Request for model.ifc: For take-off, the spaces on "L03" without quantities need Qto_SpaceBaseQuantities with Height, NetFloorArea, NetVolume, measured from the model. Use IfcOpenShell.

First a look at what the model holds.

```python
import ifcopenshell
import ifcopenshell.util.element
import ifcopenshell.util.unit

model = ifcopenshell.open("model.ifc")
print(model.schema)
for unit_type in ("LENGTHUNIT", "AREAUNIT", "VOLUMEUNIT"):
    print(unit_type, ifcopenshell.util.unit.calculate_unit_scale(model, unit_type))
storey = next(s for s in model.by_type("IfcBuildingStorey") if s.Name == "L03")
spaces = [e for e in ifcopenshell.util.element.get_decomposition(storey) if e.is_a("IfcSpace")]
for e in sorted(spaces, key=lambda e: e.id()):
    print(e.id(), e.is_a(), e.Name, list(ifcopenshell.util.element.get_psets(e, qtos_only=True)), sep=" | ")
```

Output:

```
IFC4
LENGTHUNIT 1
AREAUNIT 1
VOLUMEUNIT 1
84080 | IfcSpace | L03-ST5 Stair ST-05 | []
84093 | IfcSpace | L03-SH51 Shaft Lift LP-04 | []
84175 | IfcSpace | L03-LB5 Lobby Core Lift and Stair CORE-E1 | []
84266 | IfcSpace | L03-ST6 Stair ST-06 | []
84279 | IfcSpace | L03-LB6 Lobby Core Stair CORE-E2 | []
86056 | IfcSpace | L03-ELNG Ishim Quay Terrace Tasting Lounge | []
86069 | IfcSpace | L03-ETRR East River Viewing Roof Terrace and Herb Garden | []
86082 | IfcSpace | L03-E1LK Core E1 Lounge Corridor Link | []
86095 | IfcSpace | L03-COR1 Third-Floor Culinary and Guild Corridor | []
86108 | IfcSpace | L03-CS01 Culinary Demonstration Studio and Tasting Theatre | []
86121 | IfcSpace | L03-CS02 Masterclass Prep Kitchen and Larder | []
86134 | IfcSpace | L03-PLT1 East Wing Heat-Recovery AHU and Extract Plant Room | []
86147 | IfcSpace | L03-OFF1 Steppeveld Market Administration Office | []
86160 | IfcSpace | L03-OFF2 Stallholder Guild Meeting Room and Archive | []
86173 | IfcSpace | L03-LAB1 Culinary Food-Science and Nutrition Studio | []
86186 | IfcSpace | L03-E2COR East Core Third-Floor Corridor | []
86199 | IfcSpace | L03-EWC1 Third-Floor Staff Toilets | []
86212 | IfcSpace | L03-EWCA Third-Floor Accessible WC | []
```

```python
import ifcopenshell
import ifcopenshell.api.pset
import ifcopenshell.geom
import ifcopenshell.util.element
import ifcopenshell.util.shape
import ifcopenshell.util.unit

model = ifcopenshell.open("model.ifc")
unit_scale = ifcopenshell.util.unit.calculate_unit_scale(model)
area_scale = ifcopenshell.util.unit.calculate_unit_scale(model, "AREAUNIT")
volume_scale = ifcopenshell.util.unit.calculate_unit_scale(model, "VOLUMEUNIT")
settings = ifcopenshell.geom.settings()

storey = next(s for s in model.by_type("IfcBuildingStorey") if s.Name == "L03")
spaces = [e for e in ifcopenshell.util.element.get_decomposition(storey) if e.is_a("IfcSpace")]

for e in sorted(spaces, key=lambda e: e.id()):
    if ifcopenshell.util.element.get_psets(e, qtos_only=True, should_inherit=False):
        continue
    # Geometry comes back in metres, in the element's own axes.
    shape = ifcopenshell.geom.create_shape(settings, e)
    values = {
        "Height": ifcopenshell.util.shape.get_z(shape.geometry) / unit_scale,
        "NetFloorArea": ifcopenshell.util.shape.get_footprint_area(shape.geometry) / area_scale,
        "NetVolume": ifcopenshell.util.shape.get_volume(shape.geometry) / volume_scale,
    }
    qto = ifcopenshell.api.pset.add_qto(model, product=e, name="Qto_SpaceBaseQuantities")
    ifcopenshell.api.pset.edit_qto(model, qto=qto, properties=values)
    print(e.id(), {k: round(v, 3) for k, v in values.items()})

model.write("model_updated.ifc")
```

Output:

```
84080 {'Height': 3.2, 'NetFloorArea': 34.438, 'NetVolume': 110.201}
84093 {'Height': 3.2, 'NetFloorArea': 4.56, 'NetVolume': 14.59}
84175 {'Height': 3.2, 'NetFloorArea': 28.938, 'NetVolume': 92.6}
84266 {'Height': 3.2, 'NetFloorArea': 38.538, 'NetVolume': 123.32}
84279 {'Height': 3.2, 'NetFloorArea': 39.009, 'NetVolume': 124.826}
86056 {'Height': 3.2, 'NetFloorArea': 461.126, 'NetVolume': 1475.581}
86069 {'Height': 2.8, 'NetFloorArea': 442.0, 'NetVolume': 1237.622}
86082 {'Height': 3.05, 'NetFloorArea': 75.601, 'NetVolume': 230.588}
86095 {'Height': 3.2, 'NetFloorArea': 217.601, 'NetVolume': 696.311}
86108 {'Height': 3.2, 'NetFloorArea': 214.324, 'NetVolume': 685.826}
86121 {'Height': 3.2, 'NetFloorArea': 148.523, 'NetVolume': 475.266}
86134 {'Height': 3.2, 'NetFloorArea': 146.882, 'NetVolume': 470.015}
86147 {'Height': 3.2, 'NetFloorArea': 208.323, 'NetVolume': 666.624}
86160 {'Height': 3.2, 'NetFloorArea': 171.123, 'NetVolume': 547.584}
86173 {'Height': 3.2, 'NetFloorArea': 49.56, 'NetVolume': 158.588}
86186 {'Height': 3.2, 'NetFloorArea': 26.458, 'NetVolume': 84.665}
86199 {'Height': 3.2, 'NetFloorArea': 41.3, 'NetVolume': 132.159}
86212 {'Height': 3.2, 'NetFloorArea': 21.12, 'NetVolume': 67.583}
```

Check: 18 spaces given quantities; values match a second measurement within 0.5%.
